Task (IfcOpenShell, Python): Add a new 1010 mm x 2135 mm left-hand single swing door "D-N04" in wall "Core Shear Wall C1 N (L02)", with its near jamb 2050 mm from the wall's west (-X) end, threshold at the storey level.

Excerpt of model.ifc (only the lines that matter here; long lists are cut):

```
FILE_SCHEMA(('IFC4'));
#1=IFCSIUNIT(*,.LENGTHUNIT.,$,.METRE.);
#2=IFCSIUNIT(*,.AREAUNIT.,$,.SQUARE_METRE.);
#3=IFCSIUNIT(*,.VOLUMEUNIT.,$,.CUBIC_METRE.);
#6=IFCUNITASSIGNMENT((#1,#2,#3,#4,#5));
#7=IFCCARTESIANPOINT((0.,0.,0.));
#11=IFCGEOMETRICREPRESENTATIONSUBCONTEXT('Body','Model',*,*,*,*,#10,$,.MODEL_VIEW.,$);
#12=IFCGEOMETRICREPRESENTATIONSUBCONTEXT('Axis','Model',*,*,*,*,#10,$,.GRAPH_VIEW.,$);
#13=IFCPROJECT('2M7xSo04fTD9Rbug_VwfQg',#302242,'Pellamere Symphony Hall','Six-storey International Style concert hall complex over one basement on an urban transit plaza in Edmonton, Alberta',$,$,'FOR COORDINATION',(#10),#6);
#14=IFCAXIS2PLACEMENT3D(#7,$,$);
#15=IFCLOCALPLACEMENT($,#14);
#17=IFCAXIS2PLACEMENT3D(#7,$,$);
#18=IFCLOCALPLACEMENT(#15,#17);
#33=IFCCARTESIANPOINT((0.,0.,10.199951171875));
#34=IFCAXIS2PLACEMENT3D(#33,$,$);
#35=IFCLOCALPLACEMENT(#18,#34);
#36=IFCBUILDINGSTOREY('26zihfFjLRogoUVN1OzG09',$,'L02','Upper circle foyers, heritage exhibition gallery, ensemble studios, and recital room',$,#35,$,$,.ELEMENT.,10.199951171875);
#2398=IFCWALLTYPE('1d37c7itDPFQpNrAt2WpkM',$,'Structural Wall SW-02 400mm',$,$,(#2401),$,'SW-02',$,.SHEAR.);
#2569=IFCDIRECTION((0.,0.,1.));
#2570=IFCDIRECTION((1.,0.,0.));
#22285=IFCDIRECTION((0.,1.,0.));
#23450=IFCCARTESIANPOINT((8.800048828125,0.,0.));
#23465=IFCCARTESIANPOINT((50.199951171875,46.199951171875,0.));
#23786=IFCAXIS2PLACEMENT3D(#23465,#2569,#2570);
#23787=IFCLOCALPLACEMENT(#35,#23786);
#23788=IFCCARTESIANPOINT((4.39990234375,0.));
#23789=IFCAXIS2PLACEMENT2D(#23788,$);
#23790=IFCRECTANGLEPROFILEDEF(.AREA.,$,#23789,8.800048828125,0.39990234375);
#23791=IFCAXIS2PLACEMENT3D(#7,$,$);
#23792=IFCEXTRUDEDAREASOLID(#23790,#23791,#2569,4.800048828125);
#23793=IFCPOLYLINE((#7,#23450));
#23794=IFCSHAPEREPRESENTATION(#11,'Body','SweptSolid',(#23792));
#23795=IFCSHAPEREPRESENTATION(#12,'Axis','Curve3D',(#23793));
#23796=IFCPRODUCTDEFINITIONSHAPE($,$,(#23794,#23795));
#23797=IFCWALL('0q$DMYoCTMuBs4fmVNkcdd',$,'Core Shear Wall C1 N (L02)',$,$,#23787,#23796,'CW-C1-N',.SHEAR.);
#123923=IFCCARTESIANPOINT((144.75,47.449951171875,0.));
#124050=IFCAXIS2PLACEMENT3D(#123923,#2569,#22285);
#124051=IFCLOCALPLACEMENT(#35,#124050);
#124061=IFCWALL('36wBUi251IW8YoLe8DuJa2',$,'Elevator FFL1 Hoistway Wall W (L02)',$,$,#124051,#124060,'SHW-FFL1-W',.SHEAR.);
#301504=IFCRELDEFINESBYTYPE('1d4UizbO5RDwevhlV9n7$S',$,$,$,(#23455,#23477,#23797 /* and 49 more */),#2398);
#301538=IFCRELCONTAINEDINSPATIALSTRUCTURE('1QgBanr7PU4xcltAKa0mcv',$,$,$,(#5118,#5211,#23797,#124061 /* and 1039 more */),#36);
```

```python
import numpy as np
import ifcopenshell
import ifcopenshell.api.feature
import ifcopenshell.api.geometry
import ifcopenshell.api.root
import ifcopenshell.api.spatial
import ifcopenshell.geom
import ifcopenshell.util.element
import ifcopenshell.util.placement
import ifcopenshell.util.representation
import ifcopenshell.util.shape
import ifcopenshell.util.unit

model = ifcopenshell.open("model.ifc")
unit_scale = ifcopenshell.util.unit.calculate_unit_scale(model)
settings = ifcopenshell.geom.settings()


def volume(element):
    """Net volume in cubic metres, openings subtracted."""
    shape = ifcopenshell.geom.create_shape(settings, element)
    return ifcopenshell.util.shape.get_volume(shape.geometry)


wall = model.by_guid("0q$DMYoCTMuBs4fmVNkcdd")
storey = ifcopenshell.util.element.get_container(wall, ifc_class="IfcBuildingStorey")
context = ifcopenshell.util.representation.get_context(model, "Model", "Body", "MODEL_VIEW")
before = volume(wall)

width, height, from_end, sill = 1.01, 2.135, 2.05, 0.0  # metres

# The wall runs along its own X axis, and the end named is its -X end.
wall_shape = ifcopenshell.geom.create_shape(settings, wall)
x, y, z = ifcopenshell.util.shape.get_vertices(wall_shape.geometry).T
start = x.min() + from_end
face, thickness = float(y.min()), float(y.max() - y.min())
wall_matrix = ifcopenshell.util.placement.get_local_placement(wall.ObjectPlacement)
level = ifcopenshell.util.placement.get_local_placement(storey.ObjectPlacement)[2, 3]


def in_wall(x, y):
    """Placement at x, y metres in the wall's axes, at sill height."""
    matrix = wall_matrix.copy()
    matrix[:, 3] = wall_matrix @ np.array([x / unit_scale, y / unit_scale, 0.0, 1.0])
    matrix[2, 3] = level + sill / unit_scale
    return matrix


# Opening: a box that overshoots both wall faces by 50 mm.
opening = ifcopenshell.api.root.create_entity(model, ifc_class="IfcOpeningElement", predefined_type="OPENING")
box = ifcopenshell.api.geometry.add_wall_representation(
    model, context=context, length=width, height=height, thickness=thickness + 0.1
)
ifcopenshell.api.geometry.assign_representation(model, product=opening, representation=box)
ifcopenshell.api.geometry.edit_object_placement(model, product=opening, matrix=in_wall(start, face - 0.05), is_si=False)
ifcopenshell.api.feature.add_feature(model, feature=opening, element=wall)

door = ifcopenshell.api.root.create_entity(model, ifc_class="IfcDoor", name="D-N04", predefined_type="DOOR")
door.OverallWidth, door.OverallHeight = width / unit_scale, height / unit_scale
door.OperationType = "SINGLE_SWING_LEFT"
body = ifcopenshell.api.geometry.add_door_representation(
    model,
    context=context,
    overall_width=door.OverallWidth,
    overall_height=door.OverallHeight,
    operation_type="SINGLE_SWING_LEFT",
    lining_properties={"LiningDepth": thickness / unit_scale, "ThresholdDepth": thickness / unit_scale},
)
ifcopenshell.api.geometry.assign_representation(model, product=door, representation=body)
ifcopenshell.api.spatial.assign_container(model, products=[door], relating_structure=storey)
ifcopenshell.api.feature.add_filling(model, opening=opening, element=door)

# The lining spans the wall, so the door starts at the wall face.
ifcopenshell.api.geometry.edit_object_placement(model, product=door, matrix=in_wall(start, face), is_si=False)

after = volume(wall)

print(f"wall volume {before:.3f} -> {after:.3f} m3")

model.write("model_updated.ifc")
```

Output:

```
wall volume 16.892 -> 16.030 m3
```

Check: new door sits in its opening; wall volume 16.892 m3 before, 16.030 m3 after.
